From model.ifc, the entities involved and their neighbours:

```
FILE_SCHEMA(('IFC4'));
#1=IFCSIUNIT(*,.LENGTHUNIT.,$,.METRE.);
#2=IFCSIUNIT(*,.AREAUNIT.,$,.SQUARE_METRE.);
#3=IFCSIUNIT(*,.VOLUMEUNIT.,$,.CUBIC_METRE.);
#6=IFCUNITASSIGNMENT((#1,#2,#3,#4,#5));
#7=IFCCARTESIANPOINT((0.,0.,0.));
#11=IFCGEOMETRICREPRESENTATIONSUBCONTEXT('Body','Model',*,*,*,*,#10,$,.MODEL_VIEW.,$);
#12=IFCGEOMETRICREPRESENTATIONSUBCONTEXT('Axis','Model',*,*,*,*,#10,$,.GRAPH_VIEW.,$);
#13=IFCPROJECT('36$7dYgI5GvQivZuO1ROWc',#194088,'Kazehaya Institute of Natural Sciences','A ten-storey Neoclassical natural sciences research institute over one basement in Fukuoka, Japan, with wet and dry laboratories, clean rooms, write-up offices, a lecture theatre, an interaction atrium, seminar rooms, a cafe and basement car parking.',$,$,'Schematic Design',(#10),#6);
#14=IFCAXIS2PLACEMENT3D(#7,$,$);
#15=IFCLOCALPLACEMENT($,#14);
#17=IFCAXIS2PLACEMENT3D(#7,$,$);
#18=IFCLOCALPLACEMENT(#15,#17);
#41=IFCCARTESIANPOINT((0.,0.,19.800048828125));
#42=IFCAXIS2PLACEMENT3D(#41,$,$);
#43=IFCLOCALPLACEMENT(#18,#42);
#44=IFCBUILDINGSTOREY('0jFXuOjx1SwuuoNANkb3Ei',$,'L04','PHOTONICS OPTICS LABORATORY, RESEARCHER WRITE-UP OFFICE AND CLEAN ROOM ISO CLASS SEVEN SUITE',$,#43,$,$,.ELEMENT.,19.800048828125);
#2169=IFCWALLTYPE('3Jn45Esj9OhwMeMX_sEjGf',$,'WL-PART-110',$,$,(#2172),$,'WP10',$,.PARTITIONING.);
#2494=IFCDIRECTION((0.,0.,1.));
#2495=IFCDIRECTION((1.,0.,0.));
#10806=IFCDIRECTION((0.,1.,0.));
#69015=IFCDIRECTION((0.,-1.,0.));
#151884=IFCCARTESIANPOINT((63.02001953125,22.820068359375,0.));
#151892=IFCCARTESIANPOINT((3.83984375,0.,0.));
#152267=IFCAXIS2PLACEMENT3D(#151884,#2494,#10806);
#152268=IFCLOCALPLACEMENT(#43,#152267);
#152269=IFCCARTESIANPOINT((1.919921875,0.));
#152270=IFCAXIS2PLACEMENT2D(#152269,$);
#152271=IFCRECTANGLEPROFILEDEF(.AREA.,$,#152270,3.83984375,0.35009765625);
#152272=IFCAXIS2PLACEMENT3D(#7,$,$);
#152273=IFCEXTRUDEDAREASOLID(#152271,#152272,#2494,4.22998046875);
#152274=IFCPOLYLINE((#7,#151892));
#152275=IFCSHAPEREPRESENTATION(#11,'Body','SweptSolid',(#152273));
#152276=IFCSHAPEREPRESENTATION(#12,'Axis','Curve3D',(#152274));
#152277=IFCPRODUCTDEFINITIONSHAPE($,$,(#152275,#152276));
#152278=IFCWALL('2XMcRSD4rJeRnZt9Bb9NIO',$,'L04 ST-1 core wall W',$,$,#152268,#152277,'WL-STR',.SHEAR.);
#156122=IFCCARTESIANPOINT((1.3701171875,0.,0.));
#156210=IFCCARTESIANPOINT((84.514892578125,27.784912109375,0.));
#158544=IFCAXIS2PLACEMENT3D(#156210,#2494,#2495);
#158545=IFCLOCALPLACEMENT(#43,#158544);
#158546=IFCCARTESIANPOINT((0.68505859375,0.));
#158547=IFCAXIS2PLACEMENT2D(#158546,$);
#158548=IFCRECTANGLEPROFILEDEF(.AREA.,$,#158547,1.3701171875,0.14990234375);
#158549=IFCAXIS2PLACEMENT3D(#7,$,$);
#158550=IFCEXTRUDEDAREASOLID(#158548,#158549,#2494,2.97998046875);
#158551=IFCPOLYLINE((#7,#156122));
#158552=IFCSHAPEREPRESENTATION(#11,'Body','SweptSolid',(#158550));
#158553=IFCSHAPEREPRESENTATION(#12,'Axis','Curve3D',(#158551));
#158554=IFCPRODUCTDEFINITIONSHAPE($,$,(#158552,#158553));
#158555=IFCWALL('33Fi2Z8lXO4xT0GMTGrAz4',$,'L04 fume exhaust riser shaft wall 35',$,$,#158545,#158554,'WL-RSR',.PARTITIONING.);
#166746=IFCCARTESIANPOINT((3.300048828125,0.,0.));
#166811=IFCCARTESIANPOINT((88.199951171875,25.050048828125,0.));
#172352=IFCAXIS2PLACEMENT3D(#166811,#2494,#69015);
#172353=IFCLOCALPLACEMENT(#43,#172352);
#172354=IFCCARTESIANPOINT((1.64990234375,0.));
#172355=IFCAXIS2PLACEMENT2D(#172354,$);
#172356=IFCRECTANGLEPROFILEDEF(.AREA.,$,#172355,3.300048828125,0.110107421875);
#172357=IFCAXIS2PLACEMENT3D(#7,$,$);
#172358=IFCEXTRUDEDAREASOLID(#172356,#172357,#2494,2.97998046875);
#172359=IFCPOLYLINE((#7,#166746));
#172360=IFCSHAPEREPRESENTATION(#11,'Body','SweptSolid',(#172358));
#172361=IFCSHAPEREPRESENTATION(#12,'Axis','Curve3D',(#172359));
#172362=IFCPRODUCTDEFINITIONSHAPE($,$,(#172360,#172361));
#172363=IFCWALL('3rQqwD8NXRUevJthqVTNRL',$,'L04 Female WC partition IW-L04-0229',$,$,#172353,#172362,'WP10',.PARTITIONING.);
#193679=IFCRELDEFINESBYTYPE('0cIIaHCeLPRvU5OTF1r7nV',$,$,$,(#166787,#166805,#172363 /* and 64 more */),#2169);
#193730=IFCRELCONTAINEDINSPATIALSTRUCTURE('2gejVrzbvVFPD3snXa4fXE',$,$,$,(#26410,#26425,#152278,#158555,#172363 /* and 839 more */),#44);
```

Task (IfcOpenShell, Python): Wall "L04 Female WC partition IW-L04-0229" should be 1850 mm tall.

```python
import ifcopenshell
import ifcopenshell.geom
import ifcopenshell.util.representation
import ifcopenshell.util.shape

model = ifcopenshell.open("model.ifc")
settings = ifcopenshell.geom.settings()


def volume(element):
    """Net volume in cubic metres, openings subtracted."""
    shape = ifcopenshell.geom.create_shape(settings, element)
    return ifcopenshell.util.shape.get_volume(shape.geometry)


wall = model.by_guid("3rQqwD8NXRUevJthqVTNRL")
before = volume(wall)

body = ifcopenshell.util.representation.get_representation(wall, "Model", "Body")
solid = body.Items[0]
old_height = solid.Depth
solid.Depth = 1.85
after = volume(wall)

print(f"height {old_height:g} -> {solid.Depth:g}, volume {before:.3f} -> {after:.3f} m3")

model.write("model_rev.ifc")
```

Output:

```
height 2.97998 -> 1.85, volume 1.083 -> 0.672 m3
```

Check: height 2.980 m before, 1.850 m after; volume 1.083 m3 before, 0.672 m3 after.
